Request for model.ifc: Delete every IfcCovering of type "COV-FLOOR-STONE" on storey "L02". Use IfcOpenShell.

First a look at what the model holds.

```python
import ifcopenshell
import ifcopenshell.util.element

model = ifcopenshell.open("model.ifc")
print(model.schema)
storey = next(s for s in model.by_type("IfcBuildingStorey") if s.Name == "L02")
coverings = [e for e in ifcopenshell.util.element.get_decomposition(storey) if e.is_a("IfcCovering")]
seen = {}
for e in coverings:
    element_type = ifcopenshell.util.element.get_type(e)
    name = element_type.Name if element_type not in (None, e) else None
    seen[name] = seen.get(name, 0) + 1
for name, count in sorted(seen.items(), key=str):
    print(count, "x", name)
```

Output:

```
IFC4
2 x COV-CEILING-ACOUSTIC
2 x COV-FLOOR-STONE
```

```python
import ifcopenshell
import ifcopenshell.api.root
import ifcopenshell.util.element

model = ifcopenshell.open("model.ifc")

storey = next(s for s in model.by_type("IfcBuildingStorey") if s.Name == "L02")
coverings = [e for e in ifcopenshell.util.element.get_decomposition(storey) if e.is_a("IfcCovering")]
targets = [e for e in coverings if (t := ifcopenshell.util.element.get_type(e)) not in (None, e) and t.Name == "COV-FLOOR-STONE"]

for e in targets:
    ifcopenshell.api.root.remove_product(model, product=e)
print(len(targets), "removed")

model.write("model_updated.ifc")
```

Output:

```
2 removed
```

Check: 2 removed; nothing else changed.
